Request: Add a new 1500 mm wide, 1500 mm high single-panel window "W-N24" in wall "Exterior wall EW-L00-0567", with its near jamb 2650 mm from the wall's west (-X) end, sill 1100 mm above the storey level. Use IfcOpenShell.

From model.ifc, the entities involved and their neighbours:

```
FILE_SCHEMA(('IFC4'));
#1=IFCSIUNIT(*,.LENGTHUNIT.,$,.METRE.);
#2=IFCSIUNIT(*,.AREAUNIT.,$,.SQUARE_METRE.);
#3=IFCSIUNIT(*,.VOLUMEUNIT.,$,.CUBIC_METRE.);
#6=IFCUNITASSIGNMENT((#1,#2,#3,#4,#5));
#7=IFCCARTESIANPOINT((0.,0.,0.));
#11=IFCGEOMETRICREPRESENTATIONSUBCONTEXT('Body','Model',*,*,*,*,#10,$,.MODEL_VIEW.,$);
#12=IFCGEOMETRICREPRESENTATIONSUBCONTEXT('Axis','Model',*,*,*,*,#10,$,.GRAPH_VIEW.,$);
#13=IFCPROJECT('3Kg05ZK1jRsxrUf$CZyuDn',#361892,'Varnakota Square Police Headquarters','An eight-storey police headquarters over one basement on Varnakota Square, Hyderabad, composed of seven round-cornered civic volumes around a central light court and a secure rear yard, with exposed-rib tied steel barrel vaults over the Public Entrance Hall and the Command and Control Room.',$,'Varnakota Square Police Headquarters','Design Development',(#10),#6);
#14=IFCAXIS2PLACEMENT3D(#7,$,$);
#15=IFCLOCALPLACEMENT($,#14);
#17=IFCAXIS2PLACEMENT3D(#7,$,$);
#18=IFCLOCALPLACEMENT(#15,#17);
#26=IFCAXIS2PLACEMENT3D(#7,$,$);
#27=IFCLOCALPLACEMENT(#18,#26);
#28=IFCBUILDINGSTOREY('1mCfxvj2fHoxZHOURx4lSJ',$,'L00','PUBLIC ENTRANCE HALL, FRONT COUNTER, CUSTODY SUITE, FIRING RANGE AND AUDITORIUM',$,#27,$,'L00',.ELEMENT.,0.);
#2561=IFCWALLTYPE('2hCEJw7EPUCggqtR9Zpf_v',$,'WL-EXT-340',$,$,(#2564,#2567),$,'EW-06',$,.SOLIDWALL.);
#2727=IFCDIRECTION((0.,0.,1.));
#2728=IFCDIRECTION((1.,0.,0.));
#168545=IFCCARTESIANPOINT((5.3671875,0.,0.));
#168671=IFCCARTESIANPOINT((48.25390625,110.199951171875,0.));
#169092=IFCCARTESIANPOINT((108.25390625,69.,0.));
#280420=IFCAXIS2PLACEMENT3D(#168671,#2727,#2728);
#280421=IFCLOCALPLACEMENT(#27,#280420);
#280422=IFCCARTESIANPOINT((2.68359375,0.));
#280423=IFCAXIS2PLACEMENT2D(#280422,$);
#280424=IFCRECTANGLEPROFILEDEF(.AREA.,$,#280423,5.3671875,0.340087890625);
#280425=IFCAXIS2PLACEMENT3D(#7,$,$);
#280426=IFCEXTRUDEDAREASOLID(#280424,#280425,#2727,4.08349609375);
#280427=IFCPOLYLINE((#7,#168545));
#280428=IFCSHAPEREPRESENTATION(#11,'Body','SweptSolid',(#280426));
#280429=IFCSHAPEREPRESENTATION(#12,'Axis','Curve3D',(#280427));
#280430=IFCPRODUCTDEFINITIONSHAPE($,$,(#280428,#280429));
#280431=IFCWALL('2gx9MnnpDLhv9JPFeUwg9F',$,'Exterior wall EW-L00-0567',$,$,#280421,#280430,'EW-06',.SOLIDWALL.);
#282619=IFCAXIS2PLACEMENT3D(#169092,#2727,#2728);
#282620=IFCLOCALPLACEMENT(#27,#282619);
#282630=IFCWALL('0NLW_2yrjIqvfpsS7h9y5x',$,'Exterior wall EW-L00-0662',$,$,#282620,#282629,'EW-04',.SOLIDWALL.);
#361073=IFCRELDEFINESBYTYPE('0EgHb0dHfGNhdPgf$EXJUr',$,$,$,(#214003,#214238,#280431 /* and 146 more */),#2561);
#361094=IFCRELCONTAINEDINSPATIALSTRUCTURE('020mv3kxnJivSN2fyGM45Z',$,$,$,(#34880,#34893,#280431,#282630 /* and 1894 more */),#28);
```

```python
import numpy as np
import ifcopenshell
import ifcopenshell.api.feature
import ifcopenshell.api.geometry
import ifcopenshell.api.root
import ifcopenshell.api.spatial
import ifcopenshell.geom
import ifcopenshell.util.element
import ifcopenshell.util.placement
import ifcopenshell.util.representation
import ifcopenshell.util.shape
import ifcopenshell.util.unit

model = ifcopenshell.open("model.ifc")
unit_scale = ifcopenshell.util.unit.calculate_unit_scale(model)
settings = ifcopenshell.geom.settings()


def volume(element):
    """Net volume in cubic metres, openings subtracted."""
    shape = ifcopenshell.geom.create_shape(settings, element)
    return ifcopenshell.util.shape.get_volume(shape.geometry)


wall = model.by_guid("2gx9MnnpDLhv9JPFeUwg9F")
storey = ifcopenshell.util.element.get_container(wall, ifc_class="IfcBuildingStorey")
context = ifcopenshell.util.representation.get_context(model, "Model", "Body", "MODEL_VIEW")
before = volume(wall)

width, height, from_end, sill = 1.5, 1.5, 2.65, 1.1  # metres

# The wall runs along its own X axis, and the end named is its -X end.
wall_shape = ifcopenshell.geom.create_shape(settings, wall)
x, y, z = ifcopenshell.util.shape.get_vertices(wall_shape.geometry).T
start = x.min() + from_end
face, thickness = float(y.min()), float(y.max() - y.min())
wall_matrix = ifcopenshell.util.placement.get_local_placement(wall.ObjectPlacement)
level = ifcopenshell.util.placement.get_local_placement(storey.ObjectPlacement)[2, 3]


def in_wall(x, y):
    """Placement at x, y metres in the wall's axes, at sill height."""
    matrix = wall_matrix.copy()
    matrix[:, 3] = wall_matrix @ np.array([x / unit_scale, y / unit_scale, 0.0, 1.0])
    matrix[2, 3] = level + sill / unit_scale
    return matrix


# Opening: a box that overshoots both wall faces by 50 mm.
opening = ifcopenshell.api.root.create_entity(model, ifc_class="IfcOpeningElement", predefined_type="OPENING")
box = ifcopenshell.api.geometry.add_wall_representation(
    model, context=context, length=width, height=height, thickness=thickness + 0.1
)
ifcopenshell.api.geometry.assign_representation(model, product=opening, representation=box)
ifcopenshell.api.geometry.edit_object_placement(model, product=opening, matrix=in_wall(start, face - 0.05), is_si=False)
ifcopenshell.api.feature.add_feature(model, feature=opening, element=wall)

window = ifcopenshell.api.root.create_entity(model, ifc_class="IfcWindow", name="W-N24", predefined_type="WINDOW")
window.OverallWidth, window.OverallHeight = width / unit_scale, height / unit_scale
window.PartitioningType = "SINGLE_PANEL"
body = ifcopenshell.api.geometry.add_window_representation(
    model,
    context=context,
    overall_width=window.OverallWidth,
    overall_height=window.OverallHeight,
    partition_type="SINGLE_PANEL",
)
ifcopenshell.api.geometry.assign_representation(model, product=window, representation=body)
ifcopenshell.api.spatial.assign_container(model, products=[window], relating_structure=storey)
ifcopenshell.api.feature.add_filling(model, opening=opening, element=window)

# Centre the window in the wall's thickness.
ifcopenshell.api.geometry.edit_object_placement(model, product=window, matrix=in_wall(start, face), is_si=False)
window_shape = ifcopenshell.geom.create_shape(settings, window)
depth = ifcopenshell.util.shape.get_vertices(window_shape.geometry)[:, 1]
offset = face + thickness / 2 - (depth.min() + depth.max()) / 2
ifcopenshell.api.geometry.edit_object_placement(model, product=window, matrix=in_wall(start, offset), is_si=False)

after = volume(wall)

print(f"wall volume {before:.3f} -> {after:.3f} m3")

model.write("model_edited.ifc")
```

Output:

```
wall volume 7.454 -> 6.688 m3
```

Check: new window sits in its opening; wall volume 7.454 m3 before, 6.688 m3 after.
